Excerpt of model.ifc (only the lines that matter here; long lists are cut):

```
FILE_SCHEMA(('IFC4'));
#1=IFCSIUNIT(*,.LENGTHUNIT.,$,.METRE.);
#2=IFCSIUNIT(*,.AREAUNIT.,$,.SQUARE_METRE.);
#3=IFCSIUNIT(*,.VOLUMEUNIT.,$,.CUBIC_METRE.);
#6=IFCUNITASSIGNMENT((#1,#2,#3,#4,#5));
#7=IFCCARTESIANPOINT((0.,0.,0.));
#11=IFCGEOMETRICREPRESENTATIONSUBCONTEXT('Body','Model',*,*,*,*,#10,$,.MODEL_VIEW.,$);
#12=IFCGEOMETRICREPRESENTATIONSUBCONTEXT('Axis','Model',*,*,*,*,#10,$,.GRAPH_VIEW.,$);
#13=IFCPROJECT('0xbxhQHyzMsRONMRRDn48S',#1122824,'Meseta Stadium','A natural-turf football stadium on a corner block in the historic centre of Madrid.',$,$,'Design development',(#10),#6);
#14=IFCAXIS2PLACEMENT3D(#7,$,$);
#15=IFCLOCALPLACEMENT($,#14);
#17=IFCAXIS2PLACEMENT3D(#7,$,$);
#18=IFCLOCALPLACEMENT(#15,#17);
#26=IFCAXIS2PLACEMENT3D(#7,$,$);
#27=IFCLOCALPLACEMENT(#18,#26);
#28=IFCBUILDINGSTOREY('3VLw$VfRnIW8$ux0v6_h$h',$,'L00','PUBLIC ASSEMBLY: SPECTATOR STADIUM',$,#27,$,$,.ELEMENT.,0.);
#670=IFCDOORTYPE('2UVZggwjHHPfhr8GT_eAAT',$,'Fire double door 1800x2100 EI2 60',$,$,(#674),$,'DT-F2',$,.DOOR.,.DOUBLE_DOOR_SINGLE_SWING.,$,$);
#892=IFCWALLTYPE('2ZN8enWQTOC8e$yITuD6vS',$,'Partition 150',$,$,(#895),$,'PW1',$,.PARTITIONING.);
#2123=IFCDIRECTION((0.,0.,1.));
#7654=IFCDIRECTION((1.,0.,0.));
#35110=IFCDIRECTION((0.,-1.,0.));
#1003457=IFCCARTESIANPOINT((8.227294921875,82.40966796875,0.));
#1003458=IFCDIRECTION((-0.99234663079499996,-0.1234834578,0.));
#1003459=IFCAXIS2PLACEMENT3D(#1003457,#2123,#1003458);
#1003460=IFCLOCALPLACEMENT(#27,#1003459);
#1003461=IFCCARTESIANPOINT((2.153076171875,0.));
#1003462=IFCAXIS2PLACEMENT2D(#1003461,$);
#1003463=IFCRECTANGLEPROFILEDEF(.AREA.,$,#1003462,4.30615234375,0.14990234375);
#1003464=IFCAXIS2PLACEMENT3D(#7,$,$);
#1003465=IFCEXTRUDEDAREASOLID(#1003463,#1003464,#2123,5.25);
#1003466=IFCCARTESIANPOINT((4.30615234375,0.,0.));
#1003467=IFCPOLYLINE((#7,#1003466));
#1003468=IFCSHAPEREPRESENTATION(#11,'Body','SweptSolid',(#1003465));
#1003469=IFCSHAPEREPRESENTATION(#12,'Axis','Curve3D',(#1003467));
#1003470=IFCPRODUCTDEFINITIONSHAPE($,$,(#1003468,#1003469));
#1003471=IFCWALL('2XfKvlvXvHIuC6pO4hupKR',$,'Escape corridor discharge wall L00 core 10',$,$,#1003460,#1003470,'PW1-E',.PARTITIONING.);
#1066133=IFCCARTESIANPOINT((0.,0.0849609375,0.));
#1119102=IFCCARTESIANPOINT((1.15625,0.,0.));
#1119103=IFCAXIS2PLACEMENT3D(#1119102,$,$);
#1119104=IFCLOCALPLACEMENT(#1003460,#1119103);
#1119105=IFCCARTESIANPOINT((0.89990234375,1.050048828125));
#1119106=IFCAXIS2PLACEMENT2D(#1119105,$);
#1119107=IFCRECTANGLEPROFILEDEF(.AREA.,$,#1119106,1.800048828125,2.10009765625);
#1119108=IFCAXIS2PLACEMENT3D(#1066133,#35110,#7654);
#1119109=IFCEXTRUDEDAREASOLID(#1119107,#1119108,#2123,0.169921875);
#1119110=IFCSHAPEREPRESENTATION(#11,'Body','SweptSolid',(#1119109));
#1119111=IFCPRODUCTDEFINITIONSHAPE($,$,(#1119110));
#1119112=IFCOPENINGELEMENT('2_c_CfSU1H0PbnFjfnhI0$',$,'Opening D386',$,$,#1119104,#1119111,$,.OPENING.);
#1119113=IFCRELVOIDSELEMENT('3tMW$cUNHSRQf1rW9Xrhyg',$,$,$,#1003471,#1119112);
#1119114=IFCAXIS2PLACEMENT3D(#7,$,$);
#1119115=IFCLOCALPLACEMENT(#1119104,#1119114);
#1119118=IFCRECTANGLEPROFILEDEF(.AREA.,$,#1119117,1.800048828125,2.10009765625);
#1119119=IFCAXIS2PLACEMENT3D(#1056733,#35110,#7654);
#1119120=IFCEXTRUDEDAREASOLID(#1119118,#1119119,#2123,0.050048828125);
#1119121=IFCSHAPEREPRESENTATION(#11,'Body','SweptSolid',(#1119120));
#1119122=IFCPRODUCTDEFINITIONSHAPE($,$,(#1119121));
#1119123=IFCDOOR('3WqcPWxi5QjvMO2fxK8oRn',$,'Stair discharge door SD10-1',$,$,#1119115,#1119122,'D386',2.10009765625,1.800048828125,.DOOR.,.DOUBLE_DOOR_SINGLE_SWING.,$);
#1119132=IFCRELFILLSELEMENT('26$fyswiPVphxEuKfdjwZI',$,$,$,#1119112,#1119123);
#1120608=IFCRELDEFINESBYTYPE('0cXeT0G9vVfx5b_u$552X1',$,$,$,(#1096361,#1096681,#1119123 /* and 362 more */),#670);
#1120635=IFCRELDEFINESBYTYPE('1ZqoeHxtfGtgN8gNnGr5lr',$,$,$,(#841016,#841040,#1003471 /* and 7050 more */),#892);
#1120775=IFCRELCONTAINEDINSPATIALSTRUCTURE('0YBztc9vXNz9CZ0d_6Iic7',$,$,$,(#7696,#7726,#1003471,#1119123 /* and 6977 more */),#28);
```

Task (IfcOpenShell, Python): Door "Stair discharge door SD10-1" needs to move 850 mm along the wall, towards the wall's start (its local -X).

```python
import ifcopenshell
import ifcopenshell.api.geometry
import ifcopenshell.util.placement
import ifcopenshell.util.unit

model = ifcopenshell.open("model.ifc")
unit_scale = ifcopenshell.util.unit.calculate_unit_scale(model)

door = model.by_guid("3WqcPWxi5QjvMO2fxK8oRn")
opening = door.FillsVoids[0].RelatingOpeningElement
wall = opening.VoidsElements[0].RelatingBuildingElement

wall_matrix = ifcopenshell.util.placement.get_local_placement(wall.ObjectPlacement)
shift = wall_matrix[:3, 0] * -0.85 / unit_scale
before = ifcopenshell.util.placement.get_local_placement(door.ObjectPlacement)[:3, 3].copy()

# The door is placed relative to its opening, so it follows when the opening moves.
matrix = ifcopenshell.util.placement.get_local_placement(opening.ObjectPlacement)
matrix[:3, 3] += shift
ifcopenshell.api.geometry.edit_object_placement(
    model, product=opening, matrix=matrix, is_si=False, should_transform_children=True
)

after = ifcopenshell.util.placement.get_local_placement(door.ObjectPlacement)[:3, 3]
print("door moved by", (after - before).round(3) + 0.0)

model.write("model_updated.ifc")
```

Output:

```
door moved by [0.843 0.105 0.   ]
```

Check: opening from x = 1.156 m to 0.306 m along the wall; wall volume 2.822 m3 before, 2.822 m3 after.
